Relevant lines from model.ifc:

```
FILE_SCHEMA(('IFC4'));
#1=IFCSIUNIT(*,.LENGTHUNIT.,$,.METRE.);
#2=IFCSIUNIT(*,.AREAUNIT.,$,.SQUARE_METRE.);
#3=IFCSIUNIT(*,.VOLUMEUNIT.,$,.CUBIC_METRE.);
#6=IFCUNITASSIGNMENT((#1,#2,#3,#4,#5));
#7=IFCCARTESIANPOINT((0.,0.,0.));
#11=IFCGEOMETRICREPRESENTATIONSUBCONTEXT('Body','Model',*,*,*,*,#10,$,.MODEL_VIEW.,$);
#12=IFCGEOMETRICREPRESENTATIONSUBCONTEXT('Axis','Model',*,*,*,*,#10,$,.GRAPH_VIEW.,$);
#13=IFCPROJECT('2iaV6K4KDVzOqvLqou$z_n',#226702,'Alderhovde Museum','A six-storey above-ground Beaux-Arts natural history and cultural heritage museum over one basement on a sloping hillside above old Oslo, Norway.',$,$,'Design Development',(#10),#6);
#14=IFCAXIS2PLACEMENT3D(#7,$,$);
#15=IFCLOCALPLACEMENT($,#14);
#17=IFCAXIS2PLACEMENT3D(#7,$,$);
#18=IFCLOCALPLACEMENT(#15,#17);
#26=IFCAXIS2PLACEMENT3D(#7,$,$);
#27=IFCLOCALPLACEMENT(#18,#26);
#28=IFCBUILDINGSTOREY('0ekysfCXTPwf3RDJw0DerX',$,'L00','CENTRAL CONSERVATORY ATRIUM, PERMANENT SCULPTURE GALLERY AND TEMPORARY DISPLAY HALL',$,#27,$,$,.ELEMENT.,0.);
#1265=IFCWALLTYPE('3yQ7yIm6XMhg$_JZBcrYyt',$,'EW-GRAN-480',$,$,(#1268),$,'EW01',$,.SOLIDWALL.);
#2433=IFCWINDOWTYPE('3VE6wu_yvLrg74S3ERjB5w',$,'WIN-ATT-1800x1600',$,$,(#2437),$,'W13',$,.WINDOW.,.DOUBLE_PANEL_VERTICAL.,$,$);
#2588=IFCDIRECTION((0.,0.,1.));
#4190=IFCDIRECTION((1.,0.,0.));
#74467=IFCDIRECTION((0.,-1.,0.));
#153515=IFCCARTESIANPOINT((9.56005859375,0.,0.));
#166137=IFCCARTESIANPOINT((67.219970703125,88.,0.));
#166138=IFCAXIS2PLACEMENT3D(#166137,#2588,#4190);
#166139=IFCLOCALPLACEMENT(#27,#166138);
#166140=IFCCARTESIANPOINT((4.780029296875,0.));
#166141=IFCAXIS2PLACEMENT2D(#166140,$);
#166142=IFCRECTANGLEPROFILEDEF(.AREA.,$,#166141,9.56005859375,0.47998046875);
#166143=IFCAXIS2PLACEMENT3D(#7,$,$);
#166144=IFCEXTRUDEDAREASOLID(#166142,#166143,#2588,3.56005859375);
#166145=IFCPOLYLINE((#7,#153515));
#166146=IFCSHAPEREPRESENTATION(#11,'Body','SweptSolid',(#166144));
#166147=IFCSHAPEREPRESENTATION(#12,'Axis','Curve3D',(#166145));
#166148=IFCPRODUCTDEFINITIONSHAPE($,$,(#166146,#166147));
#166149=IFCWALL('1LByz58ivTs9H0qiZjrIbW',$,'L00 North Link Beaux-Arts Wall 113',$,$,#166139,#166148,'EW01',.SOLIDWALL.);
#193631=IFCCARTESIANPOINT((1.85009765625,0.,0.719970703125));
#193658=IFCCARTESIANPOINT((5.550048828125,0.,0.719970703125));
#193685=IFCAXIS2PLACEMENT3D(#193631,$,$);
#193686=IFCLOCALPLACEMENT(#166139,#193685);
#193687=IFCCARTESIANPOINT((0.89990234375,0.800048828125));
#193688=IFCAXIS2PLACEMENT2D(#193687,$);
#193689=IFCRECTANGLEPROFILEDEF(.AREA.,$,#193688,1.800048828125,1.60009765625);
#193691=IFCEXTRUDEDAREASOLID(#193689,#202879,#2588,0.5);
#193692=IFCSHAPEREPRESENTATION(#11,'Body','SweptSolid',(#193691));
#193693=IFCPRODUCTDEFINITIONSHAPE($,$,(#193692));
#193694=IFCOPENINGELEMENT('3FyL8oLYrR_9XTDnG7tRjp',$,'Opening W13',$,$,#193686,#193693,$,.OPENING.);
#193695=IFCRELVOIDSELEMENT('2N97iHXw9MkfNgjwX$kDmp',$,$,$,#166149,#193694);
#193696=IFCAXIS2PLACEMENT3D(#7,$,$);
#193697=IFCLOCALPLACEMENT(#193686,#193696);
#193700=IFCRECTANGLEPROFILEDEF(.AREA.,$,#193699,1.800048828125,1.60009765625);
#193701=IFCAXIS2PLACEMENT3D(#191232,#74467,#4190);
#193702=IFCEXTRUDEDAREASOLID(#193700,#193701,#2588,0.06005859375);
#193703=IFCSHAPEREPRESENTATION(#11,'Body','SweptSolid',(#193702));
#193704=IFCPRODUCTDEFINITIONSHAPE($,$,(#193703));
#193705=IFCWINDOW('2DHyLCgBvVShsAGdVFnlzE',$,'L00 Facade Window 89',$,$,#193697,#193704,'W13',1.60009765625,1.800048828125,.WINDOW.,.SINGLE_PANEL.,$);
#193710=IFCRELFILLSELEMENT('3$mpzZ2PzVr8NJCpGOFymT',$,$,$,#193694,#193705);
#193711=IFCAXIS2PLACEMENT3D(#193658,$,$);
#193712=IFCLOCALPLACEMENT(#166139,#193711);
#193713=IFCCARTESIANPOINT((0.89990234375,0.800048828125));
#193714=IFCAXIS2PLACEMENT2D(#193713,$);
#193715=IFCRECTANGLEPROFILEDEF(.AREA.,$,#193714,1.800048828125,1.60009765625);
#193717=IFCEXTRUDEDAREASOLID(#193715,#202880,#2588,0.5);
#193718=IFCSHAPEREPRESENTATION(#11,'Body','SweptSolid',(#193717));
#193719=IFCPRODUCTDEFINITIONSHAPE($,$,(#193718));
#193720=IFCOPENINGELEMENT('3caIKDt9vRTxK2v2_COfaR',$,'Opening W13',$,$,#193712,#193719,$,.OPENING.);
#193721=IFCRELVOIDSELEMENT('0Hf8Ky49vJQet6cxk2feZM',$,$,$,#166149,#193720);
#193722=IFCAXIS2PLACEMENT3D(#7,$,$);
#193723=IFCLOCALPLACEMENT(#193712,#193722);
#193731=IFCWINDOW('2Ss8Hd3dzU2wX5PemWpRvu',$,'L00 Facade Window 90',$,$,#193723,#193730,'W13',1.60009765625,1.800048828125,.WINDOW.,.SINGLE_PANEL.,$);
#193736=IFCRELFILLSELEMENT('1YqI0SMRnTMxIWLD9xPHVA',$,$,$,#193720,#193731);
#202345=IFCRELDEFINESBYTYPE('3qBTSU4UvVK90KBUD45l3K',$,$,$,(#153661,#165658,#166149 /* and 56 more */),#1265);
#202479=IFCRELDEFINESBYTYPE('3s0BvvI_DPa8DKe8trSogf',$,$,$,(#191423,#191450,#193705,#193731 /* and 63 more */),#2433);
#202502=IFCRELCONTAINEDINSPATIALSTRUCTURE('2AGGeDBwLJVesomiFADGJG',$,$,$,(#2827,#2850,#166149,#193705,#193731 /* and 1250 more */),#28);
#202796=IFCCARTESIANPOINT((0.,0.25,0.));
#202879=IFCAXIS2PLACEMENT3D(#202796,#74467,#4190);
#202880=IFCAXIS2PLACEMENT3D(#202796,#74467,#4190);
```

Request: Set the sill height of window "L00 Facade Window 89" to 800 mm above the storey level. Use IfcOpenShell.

```python
import numpy as np
import ifcopenshell
import ifcopenshell.api.geometry
import ifcopenshell.geom
import ifcopenshell.util.element
import ifcopenshell.util.placement
import ifcopenshell.util.shape
import ifcopenshell.util.unit

model = ifcopenshell.open("model.ifc")
unit_scale = ifcopenshell.util.unit.calculate_unit_scale(model)

window = model.by_guid("2DHyLCgBvVShsAGdVFnlzE")
opening = window.FillsVoids[0].RelatingOpeningElement
storey = ifcopenshell.util.element.get_container(window, ifc_class="IfcBuildingStorey")
level = ifcopenshell.util.placement.get_local_placement(storey.ObjectPlacement)[2, 3]

# The opening's origin need not be at the sill, so measure its lowest point.
shape = ifcopenshell.geom.create_shape(ifcopenshell.geom.settings(), opening)
bottom = ifcopenshell.util.shape.get_shape_bottom_elevation(shape, shape.geometry) / unit_scale
dz = level + 0.8 / unit_scale - bottom

shift = np.array([0.0, 0.0, dz])
# The window is placed relative to its opening, so it follows when the opening moves.
matrix = ifcopenshell.util.placement.get_local_placement(opening.ObjectPlacement)
matrix[:3, 3] += shift
ifcopenshell.api.geometry.edit_object_placement(
    model, product=opening, matrix=matrix, is_si=False, should_transform_children=True
)

print(f"moved by {dz * unit_scale:+.3f} m")

model.write("model_updated.ifc")
```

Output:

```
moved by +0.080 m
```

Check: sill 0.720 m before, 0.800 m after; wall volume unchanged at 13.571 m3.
